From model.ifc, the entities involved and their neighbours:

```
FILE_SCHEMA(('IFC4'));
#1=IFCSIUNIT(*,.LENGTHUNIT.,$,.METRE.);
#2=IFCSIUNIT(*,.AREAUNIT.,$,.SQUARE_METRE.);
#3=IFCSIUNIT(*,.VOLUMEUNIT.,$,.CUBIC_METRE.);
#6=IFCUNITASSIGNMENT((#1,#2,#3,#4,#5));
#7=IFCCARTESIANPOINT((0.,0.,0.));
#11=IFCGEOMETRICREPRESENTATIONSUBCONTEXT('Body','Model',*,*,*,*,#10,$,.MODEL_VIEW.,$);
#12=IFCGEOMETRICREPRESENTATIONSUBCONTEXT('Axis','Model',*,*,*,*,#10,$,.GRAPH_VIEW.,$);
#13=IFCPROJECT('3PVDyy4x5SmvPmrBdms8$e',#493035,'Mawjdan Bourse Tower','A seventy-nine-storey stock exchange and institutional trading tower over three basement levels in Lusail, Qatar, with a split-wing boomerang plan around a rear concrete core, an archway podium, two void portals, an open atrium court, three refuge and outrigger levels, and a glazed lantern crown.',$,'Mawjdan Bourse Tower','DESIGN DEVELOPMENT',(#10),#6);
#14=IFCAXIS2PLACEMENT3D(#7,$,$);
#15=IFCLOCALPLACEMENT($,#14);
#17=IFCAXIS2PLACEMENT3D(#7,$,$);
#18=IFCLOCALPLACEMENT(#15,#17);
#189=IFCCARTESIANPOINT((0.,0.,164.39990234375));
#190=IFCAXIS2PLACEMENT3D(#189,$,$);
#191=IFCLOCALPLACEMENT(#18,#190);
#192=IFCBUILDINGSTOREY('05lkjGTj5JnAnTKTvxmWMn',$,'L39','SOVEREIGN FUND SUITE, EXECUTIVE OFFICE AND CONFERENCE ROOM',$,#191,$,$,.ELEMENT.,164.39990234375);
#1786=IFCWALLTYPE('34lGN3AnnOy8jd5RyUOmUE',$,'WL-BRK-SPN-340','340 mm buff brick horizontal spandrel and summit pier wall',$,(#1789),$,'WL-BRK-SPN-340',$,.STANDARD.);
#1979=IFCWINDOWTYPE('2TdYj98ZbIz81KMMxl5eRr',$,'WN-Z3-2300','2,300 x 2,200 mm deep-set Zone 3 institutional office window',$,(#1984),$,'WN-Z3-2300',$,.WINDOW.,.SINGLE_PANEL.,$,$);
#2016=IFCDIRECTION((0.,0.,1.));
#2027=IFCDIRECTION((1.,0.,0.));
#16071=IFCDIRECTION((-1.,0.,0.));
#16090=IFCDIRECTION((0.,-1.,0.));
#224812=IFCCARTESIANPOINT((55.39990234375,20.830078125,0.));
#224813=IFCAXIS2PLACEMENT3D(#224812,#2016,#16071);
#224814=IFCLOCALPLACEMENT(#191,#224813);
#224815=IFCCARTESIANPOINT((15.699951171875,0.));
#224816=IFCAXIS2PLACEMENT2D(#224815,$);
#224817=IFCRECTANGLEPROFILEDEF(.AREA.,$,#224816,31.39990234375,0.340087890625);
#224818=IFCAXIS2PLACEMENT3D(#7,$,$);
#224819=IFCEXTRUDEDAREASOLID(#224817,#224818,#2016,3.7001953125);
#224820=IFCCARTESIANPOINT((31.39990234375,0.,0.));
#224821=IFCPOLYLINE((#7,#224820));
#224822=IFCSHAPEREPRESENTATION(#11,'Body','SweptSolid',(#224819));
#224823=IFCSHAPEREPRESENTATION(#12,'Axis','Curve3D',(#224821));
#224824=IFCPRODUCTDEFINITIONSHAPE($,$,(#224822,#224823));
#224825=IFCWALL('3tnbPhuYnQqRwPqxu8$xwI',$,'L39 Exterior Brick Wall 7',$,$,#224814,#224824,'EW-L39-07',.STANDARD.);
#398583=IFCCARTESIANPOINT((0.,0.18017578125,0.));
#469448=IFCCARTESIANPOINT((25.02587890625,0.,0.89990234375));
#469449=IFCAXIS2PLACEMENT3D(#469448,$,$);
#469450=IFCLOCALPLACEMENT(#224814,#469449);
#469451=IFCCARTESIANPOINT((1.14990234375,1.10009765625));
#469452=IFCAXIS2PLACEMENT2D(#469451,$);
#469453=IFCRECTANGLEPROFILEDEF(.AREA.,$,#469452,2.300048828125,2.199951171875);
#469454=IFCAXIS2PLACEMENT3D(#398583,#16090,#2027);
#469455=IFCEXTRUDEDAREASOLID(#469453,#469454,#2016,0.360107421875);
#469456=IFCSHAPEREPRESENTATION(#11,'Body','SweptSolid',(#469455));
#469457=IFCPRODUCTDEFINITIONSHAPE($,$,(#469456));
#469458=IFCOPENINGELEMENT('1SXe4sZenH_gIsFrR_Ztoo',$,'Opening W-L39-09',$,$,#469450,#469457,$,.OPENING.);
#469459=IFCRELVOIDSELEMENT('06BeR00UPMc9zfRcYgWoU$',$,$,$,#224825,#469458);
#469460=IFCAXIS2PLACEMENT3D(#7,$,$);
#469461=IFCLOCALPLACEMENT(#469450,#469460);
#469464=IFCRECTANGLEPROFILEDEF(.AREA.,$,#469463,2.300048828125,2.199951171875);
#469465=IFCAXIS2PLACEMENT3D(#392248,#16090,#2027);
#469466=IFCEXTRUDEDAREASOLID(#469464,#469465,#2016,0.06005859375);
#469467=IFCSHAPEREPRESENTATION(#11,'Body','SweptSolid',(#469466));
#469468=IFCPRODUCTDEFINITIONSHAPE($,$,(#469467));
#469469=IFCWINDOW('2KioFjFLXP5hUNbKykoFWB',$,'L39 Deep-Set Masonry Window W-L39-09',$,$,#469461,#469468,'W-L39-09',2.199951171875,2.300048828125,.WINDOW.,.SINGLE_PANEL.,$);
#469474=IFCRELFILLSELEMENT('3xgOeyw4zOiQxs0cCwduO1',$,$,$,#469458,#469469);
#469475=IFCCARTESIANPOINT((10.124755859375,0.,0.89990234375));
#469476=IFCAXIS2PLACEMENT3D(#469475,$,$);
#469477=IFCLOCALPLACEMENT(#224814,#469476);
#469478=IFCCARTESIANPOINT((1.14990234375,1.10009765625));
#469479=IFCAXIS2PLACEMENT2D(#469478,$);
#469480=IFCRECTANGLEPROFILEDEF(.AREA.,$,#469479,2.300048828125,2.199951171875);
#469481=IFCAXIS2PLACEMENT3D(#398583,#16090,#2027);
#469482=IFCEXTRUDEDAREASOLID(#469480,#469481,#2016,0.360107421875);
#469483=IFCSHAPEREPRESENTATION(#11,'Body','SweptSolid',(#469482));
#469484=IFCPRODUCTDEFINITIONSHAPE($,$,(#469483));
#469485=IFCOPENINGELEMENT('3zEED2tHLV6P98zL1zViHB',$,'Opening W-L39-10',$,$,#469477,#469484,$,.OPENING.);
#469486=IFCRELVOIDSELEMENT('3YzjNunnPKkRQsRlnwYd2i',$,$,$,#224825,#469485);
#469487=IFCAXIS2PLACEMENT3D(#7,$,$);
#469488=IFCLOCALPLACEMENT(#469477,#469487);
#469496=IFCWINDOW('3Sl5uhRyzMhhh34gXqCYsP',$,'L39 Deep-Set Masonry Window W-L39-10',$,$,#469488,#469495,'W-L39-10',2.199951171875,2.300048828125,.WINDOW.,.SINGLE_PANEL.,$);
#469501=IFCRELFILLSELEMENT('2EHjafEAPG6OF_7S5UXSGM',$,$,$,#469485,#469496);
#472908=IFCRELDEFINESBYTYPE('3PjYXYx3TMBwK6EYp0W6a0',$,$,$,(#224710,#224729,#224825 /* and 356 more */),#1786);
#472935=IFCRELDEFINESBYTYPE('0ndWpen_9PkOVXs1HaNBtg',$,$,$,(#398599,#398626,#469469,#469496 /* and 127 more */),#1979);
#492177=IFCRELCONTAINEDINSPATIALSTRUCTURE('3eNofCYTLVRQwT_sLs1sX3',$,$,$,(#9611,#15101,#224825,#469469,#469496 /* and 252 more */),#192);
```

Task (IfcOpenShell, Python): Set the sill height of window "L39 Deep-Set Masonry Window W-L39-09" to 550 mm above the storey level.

```python
import numpy as np
import ifcopenshell
import ifcopenshell.api.geometry
import ifcopenshell.geom
import ifcopenshell.util.element
import ifcopenshell.util.placement
import ifcopenshell.util.shape
import ifcopenshell.util.unit

model = ifcopenshell.open("model.ifc")
unit_scale = ifcopenshell.util.unit.calculate_unit_scale(model)

window = model.by_guid("2KioFjFLXP5hUNbKykoFWB")
opening = window.FillsVoids[0].RelatingOpeningElement
storey = ifcopenshell.util.element.get_container(window, ifc_class="IfcBuildingStorey")
level = ifcopenshell.util.placement.get_local_placement(storey.ObjectPlacement)[2, 3]

# The opening's origin need not be at the sill, so measure its lowest point.
shape = ifcopenshell.geom.create_shape(ifcopenshell.geom.settings(), opening)
bottom = ifcopenshell.util.shape.get_shape_bottom_elevation(shape, shape.geometry) / unit_scale
dz = level + 0.55 - bottom

shift = np.array([0.0, 0.0, dz])
# The window is placed relative to its opening, so it follows when the opening moves.
matrix = ifcopenshell.util.placement.get_local_placement(opening.ObjectPlacement)
matrix[:3, 3] += shift
ifcopenshell.api.geometry.edit_object_placement(
    model, product=opening, matrix=matrix, is_si=False, should_transform_children=True
)

print(f"moved by {dz * unit_scale:+.3f} m")

model.write("model_rev.ifc")
```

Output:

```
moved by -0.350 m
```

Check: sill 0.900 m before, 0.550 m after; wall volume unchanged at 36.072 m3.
